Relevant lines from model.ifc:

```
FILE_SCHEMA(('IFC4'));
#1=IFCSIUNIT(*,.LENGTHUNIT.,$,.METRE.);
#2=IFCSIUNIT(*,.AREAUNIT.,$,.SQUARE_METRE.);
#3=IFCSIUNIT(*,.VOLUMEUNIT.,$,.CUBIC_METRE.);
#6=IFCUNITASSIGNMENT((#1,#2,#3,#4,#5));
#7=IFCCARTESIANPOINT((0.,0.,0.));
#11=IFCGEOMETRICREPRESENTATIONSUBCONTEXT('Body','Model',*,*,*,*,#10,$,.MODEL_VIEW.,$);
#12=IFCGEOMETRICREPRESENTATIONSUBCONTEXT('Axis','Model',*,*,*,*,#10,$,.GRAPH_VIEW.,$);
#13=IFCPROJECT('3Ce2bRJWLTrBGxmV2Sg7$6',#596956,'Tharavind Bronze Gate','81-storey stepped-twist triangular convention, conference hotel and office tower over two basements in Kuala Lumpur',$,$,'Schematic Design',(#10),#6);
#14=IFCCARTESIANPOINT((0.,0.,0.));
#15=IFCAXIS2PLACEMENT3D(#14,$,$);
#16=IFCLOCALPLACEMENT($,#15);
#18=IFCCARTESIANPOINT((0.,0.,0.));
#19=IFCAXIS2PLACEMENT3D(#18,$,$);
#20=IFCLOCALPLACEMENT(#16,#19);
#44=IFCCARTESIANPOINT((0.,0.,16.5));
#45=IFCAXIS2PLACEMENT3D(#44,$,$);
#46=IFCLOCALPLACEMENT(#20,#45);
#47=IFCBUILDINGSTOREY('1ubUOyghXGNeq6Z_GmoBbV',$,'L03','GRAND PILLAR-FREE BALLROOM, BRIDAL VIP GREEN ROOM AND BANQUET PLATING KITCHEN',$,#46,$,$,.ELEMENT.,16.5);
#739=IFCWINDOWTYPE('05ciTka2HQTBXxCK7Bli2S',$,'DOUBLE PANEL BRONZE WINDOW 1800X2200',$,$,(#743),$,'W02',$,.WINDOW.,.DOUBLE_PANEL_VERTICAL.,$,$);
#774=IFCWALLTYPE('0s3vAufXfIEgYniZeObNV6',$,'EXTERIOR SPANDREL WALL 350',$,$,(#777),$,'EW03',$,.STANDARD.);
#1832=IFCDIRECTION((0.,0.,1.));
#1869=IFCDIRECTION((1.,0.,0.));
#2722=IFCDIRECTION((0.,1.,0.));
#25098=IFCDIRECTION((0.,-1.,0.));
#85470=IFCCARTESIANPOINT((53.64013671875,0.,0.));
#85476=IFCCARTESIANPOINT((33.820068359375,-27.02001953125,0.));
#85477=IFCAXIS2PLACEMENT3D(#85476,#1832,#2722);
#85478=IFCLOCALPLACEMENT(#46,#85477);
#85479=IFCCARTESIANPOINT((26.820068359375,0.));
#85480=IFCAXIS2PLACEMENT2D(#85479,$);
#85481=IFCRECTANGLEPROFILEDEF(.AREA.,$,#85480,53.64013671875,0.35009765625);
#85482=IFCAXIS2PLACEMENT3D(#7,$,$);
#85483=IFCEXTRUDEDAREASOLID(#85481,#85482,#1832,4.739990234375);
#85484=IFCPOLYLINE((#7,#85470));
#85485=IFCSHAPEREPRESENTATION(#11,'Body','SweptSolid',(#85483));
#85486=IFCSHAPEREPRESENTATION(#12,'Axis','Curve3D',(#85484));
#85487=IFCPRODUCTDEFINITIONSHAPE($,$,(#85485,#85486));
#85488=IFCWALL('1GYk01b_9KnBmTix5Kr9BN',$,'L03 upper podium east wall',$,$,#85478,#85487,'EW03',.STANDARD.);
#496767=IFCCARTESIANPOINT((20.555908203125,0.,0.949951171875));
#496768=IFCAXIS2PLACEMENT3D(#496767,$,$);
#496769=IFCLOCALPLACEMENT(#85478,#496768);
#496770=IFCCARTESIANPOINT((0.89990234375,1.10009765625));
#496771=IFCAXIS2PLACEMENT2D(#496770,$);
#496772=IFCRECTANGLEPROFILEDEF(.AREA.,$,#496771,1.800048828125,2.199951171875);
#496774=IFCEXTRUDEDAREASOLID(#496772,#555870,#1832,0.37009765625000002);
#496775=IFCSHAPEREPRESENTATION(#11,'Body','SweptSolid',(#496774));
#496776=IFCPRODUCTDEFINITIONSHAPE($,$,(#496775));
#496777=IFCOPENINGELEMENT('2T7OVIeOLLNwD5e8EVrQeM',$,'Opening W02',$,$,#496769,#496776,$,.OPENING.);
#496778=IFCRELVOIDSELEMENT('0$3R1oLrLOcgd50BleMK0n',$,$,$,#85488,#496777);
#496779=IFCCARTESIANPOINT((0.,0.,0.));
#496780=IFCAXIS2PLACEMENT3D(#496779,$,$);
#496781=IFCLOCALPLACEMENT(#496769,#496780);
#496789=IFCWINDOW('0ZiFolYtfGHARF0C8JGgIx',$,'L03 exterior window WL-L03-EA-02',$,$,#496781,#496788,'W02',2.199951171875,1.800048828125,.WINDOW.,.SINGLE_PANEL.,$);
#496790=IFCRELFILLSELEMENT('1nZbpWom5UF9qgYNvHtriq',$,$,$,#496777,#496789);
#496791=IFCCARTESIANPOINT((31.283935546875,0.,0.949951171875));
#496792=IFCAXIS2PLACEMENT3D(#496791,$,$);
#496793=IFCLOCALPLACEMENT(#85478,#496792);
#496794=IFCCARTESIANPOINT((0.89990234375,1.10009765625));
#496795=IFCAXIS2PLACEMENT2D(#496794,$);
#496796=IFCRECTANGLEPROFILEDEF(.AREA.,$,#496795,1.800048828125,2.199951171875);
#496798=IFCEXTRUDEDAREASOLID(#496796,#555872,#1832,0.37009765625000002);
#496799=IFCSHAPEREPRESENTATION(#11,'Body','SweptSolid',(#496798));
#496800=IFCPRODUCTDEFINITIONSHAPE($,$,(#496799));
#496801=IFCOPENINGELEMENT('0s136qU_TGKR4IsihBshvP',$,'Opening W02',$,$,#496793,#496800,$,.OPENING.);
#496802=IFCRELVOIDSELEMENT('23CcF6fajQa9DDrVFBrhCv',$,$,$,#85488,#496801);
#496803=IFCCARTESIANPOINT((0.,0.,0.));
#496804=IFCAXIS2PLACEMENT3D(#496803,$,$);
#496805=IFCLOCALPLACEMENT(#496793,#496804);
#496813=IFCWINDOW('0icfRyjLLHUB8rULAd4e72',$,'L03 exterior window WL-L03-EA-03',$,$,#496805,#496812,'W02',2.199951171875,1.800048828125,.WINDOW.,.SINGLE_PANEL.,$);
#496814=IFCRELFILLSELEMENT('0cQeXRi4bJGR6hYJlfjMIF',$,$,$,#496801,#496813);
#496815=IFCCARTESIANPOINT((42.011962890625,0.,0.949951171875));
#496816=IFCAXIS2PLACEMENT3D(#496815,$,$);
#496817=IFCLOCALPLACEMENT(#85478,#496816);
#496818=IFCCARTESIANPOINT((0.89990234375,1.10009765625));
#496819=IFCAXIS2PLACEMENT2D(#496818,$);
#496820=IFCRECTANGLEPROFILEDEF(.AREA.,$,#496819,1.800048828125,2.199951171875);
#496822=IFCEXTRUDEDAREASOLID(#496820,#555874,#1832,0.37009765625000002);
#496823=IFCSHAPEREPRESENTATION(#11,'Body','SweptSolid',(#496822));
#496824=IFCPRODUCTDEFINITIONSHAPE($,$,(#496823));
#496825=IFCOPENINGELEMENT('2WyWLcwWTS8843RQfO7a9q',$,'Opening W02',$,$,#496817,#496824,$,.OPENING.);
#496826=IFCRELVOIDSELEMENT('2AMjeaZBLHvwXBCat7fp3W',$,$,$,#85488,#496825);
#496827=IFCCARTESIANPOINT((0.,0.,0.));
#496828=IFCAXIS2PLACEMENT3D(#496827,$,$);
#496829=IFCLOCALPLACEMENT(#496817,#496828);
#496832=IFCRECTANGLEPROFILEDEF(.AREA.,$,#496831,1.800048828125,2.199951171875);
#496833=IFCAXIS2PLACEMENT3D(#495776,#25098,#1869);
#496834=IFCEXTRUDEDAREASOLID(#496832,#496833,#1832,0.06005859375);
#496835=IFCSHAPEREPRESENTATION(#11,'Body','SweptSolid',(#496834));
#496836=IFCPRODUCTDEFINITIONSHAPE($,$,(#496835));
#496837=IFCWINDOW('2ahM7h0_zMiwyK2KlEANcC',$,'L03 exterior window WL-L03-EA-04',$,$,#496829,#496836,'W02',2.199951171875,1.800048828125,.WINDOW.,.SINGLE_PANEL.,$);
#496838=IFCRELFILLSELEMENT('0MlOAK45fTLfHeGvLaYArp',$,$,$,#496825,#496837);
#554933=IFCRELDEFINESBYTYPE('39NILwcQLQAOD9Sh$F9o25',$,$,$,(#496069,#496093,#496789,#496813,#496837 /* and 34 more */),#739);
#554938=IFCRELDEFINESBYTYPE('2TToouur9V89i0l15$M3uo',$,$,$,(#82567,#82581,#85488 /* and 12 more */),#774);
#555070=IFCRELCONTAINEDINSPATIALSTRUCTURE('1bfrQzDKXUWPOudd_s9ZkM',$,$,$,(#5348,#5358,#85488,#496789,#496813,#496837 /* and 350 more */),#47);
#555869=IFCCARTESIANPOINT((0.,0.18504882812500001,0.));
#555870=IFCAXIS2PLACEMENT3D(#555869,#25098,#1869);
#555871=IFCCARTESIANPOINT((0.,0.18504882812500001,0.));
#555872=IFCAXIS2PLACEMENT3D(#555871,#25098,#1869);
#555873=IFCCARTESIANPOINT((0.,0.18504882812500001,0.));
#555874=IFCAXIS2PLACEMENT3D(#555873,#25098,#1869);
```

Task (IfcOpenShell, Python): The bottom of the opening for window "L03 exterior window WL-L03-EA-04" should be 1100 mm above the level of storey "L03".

```python
import numpy as np
import ifcopenshell
import ifcopenshell.api.geometry
import ifcopenshell.geom
import ifcopenshell.util.element
import ifcopenshell.util.placement
import ifcopenshell.util.shape
import ifcopenshell.util.unit

model = ifcopenshell.open("model.ifc")
unit_scale = ifcopenshell.util.unit.calculate_unit_scale(model)

window = model.by_id(496837)
opening = window.FillsVoids[0].RelatingOpeningElement
storey = ifcopenshell.util.element.get_container(window, ifc_class="IfcBuildingStorey")
level = ifcopenshell.util.placement.get_local_placement(storey.ObjectPlacement)[2, 3]

# The opening's origin need not be at the sill, so measure its lowest point.
shape = ifcopenshell.geom.create_shape(ifcopenshell.geom.settings(), opening)
bottom = ifcopenshell.util.shape.get_shape_bottom_elevation(shape, shape.geometry) / unit_scale
dz = level + 1.1 / unit_scale - bottom

shift = np.array([0.0, 0.0, dz])
# The window is placed relative to its opening, so it follows when the opening moves.
matrix = ifcopenshell.util.placement.get_local_placement(opening.ObjectPlacement)
matrix[:3, 3] += shift
ifcopenshell.api.geometry.edit_object_placement(
    model, product=opening, matrix=matrix, is_si=False, should_transform_children=True
)

print(f"moved by {dz * unit_scale:+.3f} m")

model.write("model_edited.ifc")
```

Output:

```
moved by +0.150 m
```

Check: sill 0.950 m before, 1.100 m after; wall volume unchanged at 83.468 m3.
